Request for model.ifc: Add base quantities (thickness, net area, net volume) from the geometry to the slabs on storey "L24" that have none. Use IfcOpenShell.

First a look at what the model holds.

```python
import ifcopenshell
import ifcopenshell.util.element
import ifcopenshell.util.unit

model = ifcopenshell.open("model.ifc")
print(model.schema)
for unit_type in ("LENGTHUNIT", "AREAUNIT", "VOLUMEUNIT"):
    print(unit_type, ifcopenshell.util.unit.calculate_unit_scale(model, unit_type))
storey = next(s for s in model.by_type("IfcBuildingStorey") if s.Name == "L24")
slabs = [e for e in ifcopenshell.util.element.get_decomposition(storey) if e.is_a("IfcSlab")]
for e in sorted(slabs, key=lambda e: e.id()):
    print(e.id(), e.is_a(), e.Name, list(ifcopenshell.util.element.get_psets(e, qtos_only=True)), sep=" | ")
```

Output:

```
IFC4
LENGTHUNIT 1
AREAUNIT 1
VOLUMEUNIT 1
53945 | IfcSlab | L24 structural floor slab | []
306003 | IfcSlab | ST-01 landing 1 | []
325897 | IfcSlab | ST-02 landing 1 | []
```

```python
import ifcopenshell
import ifcopenshell.api.pset
import ifcopenshell.geom
import ifcopenshell.util.element
import ifcopenshell.util.shape
import ifcopenshell.util.unit

model = ifcopenshell.open("model.ifc")
unit_scale = ifcopenshell.util.unit.calculate_unit_scale(model)
area_scale = ifcopenshell.util.unit.calculate_unit_scale(model, "AREAUNIT")
volume_scale = ifcopenshell.util.unit.calculate_unit_scale(model, "VOLUMEUNIT")
settings = ifcopenshell.geom.settings()

storey = next(s for s in model.by_type("IfcBuildingStorey") if s.Name == "L24")
slabs = [e for e in ifcopenshell.util.element.get_decomposition(storey) if e.is_a("IfcSlab")]

for e in sorted(slabs, key=lambda e: e.id()):
    if ifcopenshell.util.element.get_psets(e, qtos_only=True, should_inherit=False):
        continue
    # Geometry comes back in metres, in the element's own axes.
    shape = ifcopenshell.geom.create_shape(settings, e)
    values = {
        "Width": ifcopenshell.util.shape.get_z(shape.geometry) / unit_scale,
        "NetArea": ifcopenshell.util.shape.get_footprint_area(shape.geometry) / area_scale,
        "NetVolume": ifcopenshell.util.shape.get_volume(shape.geometry) / volume_scale,
    }
    qto = ifcopenshell.api.pset.add_qto(model, product=e, name="Qto_SlabBaseQuantities")
    ifcopenshell.api.pset.edit_qto(model, qto=qto, properties=values)
    print(e.id(), {k: round(v, 3) for k, v in values.items()})

model.write("model_v2.ifc")
```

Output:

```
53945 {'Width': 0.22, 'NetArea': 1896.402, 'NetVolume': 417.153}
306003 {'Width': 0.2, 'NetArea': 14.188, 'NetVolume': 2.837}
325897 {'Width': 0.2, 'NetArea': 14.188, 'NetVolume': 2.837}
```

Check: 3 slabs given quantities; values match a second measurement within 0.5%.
